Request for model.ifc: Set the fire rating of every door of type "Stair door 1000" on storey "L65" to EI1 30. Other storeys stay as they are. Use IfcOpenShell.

First a look at what the model holds.

```python
import ifcopenshell
import ifcopenshell.util.element

model = ifcopenshell.open("model.ifc")
print(model.schema)
storey = next(s for s in model.by_type("IfcBuildingStorey") if s.Name == "L65")
doors = [e for e in ifcopenshell.util.element.get_decomposition(storey) if e.is_a("IfcDoor")]
seen = {}
for e in doors:
    element_type = ifcopenshell.util.element.get_type(e)
    key = (element_type.Name if element_type != e and element_type else None, ifcopenshell.util.element.get_pset(e, "Pset_DoorCommon", "FireRating"))
    seen[key] = seen.get(key, 0) + 1
for (name, value), count in sorted(seen.items(), key=str):
    print(count, "x", name, "|", value)
```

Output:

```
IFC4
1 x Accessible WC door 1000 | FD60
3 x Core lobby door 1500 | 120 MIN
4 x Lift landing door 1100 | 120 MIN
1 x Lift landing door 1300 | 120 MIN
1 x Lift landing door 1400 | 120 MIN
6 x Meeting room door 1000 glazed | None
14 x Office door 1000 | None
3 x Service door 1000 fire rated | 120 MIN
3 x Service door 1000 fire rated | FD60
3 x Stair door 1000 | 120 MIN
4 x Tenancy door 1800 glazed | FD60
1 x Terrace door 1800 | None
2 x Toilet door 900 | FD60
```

```python
import ifcopenshell
import ifcopenshell.api.pset
import ifcopenshell.util.element

model = ifcopenshell.open("model.ifc")

storey = next(s for s in model.by_type("IfcBuildingStorey") if s.Name == "L65")
doors = [e for e in ifcopenshell.util.element.get_decomposition(storey) if e.is_a("IfcDoor")]

count = 0
for e in doors:
    element_type = ifcopenshell.util.element.get_type(e)
    if element_type in (None, e) or element_type.Name != "Stair door 1000":
        continue
    # add_pset returns the element's existing set when there is one.
    pset = ifcopenshell.api.pset.add_pset(model, product=e, name="Pset_DoorCommon")
    ifcopenshell.api.pset.edit_pset(model, pset=pset, properties={"FireRating": "EI1 30"})
    count += 1

print(count, "doors updated")

model.write("model_rev.ifc")
```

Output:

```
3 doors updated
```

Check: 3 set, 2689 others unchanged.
